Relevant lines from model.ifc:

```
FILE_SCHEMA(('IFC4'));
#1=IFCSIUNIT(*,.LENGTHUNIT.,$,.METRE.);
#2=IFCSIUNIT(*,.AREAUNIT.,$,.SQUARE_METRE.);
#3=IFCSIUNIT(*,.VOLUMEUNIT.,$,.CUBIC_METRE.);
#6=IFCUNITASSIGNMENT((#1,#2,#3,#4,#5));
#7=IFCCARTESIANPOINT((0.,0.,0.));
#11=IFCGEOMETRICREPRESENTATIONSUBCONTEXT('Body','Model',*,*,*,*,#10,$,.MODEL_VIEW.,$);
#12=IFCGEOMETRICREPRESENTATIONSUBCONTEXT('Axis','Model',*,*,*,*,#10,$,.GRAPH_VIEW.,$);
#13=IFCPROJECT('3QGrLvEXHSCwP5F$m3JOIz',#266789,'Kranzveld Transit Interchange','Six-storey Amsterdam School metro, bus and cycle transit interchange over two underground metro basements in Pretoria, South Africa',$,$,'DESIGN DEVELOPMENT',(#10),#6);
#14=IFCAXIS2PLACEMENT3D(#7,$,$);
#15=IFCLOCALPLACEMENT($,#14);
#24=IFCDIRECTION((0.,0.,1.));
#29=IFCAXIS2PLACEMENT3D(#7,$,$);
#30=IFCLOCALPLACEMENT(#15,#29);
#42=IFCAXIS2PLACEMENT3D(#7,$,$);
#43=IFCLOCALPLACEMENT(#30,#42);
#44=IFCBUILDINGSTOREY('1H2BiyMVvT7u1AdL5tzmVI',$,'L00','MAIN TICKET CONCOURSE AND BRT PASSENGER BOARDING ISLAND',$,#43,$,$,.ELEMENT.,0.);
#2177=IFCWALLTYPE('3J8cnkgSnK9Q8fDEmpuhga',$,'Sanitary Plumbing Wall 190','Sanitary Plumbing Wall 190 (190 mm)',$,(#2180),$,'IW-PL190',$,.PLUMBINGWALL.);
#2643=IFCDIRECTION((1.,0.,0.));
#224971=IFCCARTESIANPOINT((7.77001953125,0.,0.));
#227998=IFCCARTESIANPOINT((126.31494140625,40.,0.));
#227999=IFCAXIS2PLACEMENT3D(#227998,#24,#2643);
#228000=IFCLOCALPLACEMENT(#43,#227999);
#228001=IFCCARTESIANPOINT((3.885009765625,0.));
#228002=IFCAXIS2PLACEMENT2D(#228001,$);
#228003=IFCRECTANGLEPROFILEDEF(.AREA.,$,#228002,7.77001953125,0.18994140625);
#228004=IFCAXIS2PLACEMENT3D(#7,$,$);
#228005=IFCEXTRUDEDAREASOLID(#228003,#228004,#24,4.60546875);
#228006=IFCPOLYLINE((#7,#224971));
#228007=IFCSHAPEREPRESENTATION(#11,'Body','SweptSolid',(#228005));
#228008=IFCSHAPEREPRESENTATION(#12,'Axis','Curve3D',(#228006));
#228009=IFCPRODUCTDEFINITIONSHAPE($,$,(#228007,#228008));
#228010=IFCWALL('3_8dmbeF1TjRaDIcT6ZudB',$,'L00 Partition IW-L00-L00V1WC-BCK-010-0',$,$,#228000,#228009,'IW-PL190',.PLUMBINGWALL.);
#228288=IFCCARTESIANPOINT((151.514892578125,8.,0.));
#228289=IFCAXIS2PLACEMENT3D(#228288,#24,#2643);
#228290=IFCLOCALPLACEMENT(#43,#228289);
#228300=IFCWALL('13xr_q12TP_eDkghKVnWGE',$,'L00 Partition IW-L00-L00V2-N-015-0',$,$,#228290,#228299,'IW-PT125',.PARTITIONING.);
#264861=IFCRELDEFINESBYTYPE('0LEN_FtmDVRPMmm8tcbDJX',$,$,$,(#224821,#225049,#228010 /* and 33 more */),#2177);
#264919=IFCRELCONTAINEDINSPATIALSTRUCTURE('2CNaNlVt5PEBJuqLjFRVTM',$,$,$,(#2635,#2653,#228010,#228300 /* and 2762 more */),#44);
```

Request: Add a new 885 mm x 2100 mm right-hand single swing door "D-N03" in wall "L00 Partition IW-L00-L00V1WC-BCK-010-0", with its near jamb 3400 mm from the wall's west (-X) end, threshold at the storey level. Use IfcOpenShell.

```python
import numpy as np
import ifcopenshell
import ifcopenshell.api.feature
import ifcopenshell.api.geometry
import ifcopenshell.api.root
import ifcopenshell.api.spatial
import ifcopenshell.geom
import ifcopenshell.util.element
import ifcopenshell.util.placement
import ifcopenshell.util.representation
import ifcopenshell.util.shape
import ifcopenshell.util.unit

model = ifcopenshell.open("model.ifc")
unit_scale = ifcopenshell.util.unit.calculate_unit_scale(model)
settings = ifcopenshell.geom.settings()


def volume(element):
    """Net volume in cubic metres, openings subtracted."""
    shape = ifcopenshell.geom.create_shape(settings, element)
    return ifcopenshell.util.shape.get_volume(shape.geometry)


wall = model.by_guid("3_8dmbeF1TjRaDIcT6ZudB")
storey = ifcopenshell.util.element.get_container(wall, ifc_class="IfcBuildingStorey")
context = ifcopenshell.util.representation.get_context(model, "Model", "Body", "MODEL_VIEW")
before = volume(wall)

width, height, from_end, sill = 0.885, 2.1, 3.4, 0.0  # metres

# The wall runs along its own X axis, and the end named is its -X end.
wall_shape = ifcopenshell.geom.create_shape(settings, wall)
x, y, z = ifcopenshell.util.shape.get_vertices(wall_shape.geometry).T
start = x.min() + from_end
face, thickness = float(y.min()), float(y.max() - y.min())
wall_matrix = ifcopenshell.util.placement.get_local_placement(wall.ObjectPlacement)
level = ifcopenshell.util.placement.get_local_placement(storey.ObjectPlacement)[2, 3]


def in_wall(x, y):
    """Placement at x, y metres in the wall's axes, at sill height."""
    matrix = wall_matrix.copy()
    matrix[:, 3] = wall_matrix @ np.array([x / unit_scale, y / unit_scale, 0.0, 1.0])
    matrix[2, 3] = level + sill / unit_scale
    return matrix


# Opening: a box that overshoots both wall faces by 50 mm.
opening = ifcopenshell.api.root.create_entity(model, ifc_class="IfcOpeningElement", predefined_type="OPENING")
box = ifcopenshell.api.geometry.add_wall_representation(
    model, context=context, length=width, height=height, thickness=thickness + 0.1
)
ifcopenshell.api.geometry.assign_representation(model, product=opening, representation=box)
ifcopenshell.api.geometry.edit_object_placement(model, product=opening, matrix=in_wall(start, face - 0.05), is_si=False)
ifcopenshell.api.feature.add_feature(model, feature=opening, element=wall)

door = ifcopenshell.api.root.create_entity(model, ifc_class="IfcDoor", name="D-N03", predefined_type="DOOR")
door.OverallWidth, door.OverallHeight = width / unit_scale, height / unit_scale
door.OperationType = "SINGLE_SWING_RIGHT"
body = ifcopenshell.api.geometry.add_door_representation(
    model,
    context=context,
    overall_width=door.OverallWidth,
    overall_height=door.OverallHeight,
    operation_type="SINGLE_SWING_RIGHT",
    lining_properties={"LiningDepth": thickness / unit_scale, "ThresholdDepth": thickness / unit_scale},
)
ifcopenshell.api.geometry.assign_representation(model, product=door, representation=body)
ifcopenshell.api.spatial.assign_container(model, products=[door], relating_structure=storey)
ifcopenshell.api.feature.add_filling(model, opening=opening, element=door)

# The lining spans the wall, so the door starts at the wall face.
ifcopenshell.api.geometry.edit_object_placement(model, product=door, matrix=in_wall(start, face), is_si=False)

after = volume(wall)

print(f"wall volume {before:.3f} -> {after:.3f} m3")

model.write("model_edited.ifc")
```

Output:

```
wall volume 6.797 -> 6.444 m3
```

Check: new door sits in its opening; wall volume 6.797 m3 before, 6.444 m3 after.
